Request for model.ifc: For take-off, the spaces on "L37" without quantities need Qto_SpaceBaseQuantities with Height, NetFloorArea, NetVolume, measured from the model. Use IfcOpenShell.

First a look at what the model holds.

```python
import ifcopenshell
import ifcopenshell.util.element
import ifcopenshell.util.unit

model = ifcopenshell.open("model.ifc")
print(model.schema)
for unit_type in ("LENGTHUNIT", "AREAUNIT", "VOLUMEUNIT"):
    print(unit_type, ifcopenshell.util.unit.calculate_unit_scale(model, unit_type))
storey = next(s for s in model.by_type("IfcBuildingStorey") if s.Name == "L37")
spaces = [e for e in ifcopenshell.util.element.get_decomposition(storey) if e.is_a("IfcSpace")]
for e in sorted(spaces, key=lambda e: e.id()):
    print(e.id(), e.is_a(), e.Name, list(ifcopenshell.util.element.get_psets(e, qtos_only=True)), sep=" | ")
```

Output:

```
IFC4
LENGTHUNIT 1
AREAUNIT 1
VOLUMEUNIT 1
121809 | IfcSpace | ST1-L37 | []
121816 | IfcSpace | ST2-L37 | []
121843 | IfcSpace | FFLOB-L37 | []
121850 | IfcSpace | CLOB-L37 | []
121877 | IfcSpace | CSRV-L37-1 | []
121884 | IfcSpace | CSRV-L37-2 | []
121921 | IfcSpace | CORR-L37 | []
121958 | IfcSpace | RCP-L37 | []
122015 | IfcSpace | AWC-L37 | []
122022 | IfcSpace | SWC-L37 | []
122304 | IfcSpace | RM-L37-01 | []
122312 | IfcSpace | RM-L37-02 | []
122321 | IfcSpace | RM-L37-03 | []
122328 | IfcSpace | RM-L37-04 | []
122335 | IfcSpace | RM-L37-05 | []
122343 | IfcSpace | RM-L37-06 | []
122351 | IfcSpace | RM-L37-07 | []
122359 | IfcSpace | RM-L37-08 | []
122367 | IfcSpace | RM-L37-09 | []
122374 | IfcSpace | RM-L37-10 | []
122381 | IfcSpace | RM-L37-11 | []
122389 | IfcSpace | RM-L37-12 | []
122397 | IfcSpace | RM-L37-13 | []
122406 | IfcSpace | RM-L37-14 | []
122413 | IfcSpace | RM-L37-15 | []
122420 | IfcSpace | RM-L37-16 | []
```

```python
import ifcopenshell
import ifcopenshell.api.pset
import ifcopenshell.geom
import ifcopenshell.util.element
import ifcopenshell.util.shape
import ifcopenshell.util.unit

model = ifcopenshell.open("model.ifc")
unit_scale = ifcopenshell.util.unit.calculate_unit_scale(model)
area_scale = ifcopenshell.util.unit.calculate_unit_scale(model, "AREAUNIT")
volume_scale = ifcopenshell.util.unit.calculate_unit_scale(model, "VOLUMEUNIT")
settings = ifcopenshell.geom.settings()

storey = next(s for s in model.by_type("IfcBuildingStorey") if s.Name == "L37")
spaces = [e for e in ifcopenshell.util.element.get_decomposition(storey) if e.is_a("IfcSpace")]

for e in sorted(spaces, key=lambda e: e.id()):
    if ifcopenshell.util.element.get_psets(e, qtos_only=True, should_inherit=False):
        continue
    # Geometry comes back in metres, in the element's own axes.
    shape = ifcopenshell.geom.create_shape(settings, e)
    values = {
        "Height": ifcopenshell.util.shape.get_z(shape.geometry) / unit_scale,
        "NetFloorArea": ifcopenshell.util.shape.get_footprint_area(shape.geometry) / area_scale,
        "NetVolume": ifcopenshell.util.shape.get_volume(shape.geometry) / volume_scale,
    }
    qto = ifcopenshell.api.pset.add_qto(model, product=e, name="Qto_SpaceBaseQuantities")
    ifcopenshell.api.pset.edit_qto(model, qto=qto, properties=values)
    print(e.id(), {k: round(v, 3) for k, v in values.items()})

model.write("model_edited.ifc")
```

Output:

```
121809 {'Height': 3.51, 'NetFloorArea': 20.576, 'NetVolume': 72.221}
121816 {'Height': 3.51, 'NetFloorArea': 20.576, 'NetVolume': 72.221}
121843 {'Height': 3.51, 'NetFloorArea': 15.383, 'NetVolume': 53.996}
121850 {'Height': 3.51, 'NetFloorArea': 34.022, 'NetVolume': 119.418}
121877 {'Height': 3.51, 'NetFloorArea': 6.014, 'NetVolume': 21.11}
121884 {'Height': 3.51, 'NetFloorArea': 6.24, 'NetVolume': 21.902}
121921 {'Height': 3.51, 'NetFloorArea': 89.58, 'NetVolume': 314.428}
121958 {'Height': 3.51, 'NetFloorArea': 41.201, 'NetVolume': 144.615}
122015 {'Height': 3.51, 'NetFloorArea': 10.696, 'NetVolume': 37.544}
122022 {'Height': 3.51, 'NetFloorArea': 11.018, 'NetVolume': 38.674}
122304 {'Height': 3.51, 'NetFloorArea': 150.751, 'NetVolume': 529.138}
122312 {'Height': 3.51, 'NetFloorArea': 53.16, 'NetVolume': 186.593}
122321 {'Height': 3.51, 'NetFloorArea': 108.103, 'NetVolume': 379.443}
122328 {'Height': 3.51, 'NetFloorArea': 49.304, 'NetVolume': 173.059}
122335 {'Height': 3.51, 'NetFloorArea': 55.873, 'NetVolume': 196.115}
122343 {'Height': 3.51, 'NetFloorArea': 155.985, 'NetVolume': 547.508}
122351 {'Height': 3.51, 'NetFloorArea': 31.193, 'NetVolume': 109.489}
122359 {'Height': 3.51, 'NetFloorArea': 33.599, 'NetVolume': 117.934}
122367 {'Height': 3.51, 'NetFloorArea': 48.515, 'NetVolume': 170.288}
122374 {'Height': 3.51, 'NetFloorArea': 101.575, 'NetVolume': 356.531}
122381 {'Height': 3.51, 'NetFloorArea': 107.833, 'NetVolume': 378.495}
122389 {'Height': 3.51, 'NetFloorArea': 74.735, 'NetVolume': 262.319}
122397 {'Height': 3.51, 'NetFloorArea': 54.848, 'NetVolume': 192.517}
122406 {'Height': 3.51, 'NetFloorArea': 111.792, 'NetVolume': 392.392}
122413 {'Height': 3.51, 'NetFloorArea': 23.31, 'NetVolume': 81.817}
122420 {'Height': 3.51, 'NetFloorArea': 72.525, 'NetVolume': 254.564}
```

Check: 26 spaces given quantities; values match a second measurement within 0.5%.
